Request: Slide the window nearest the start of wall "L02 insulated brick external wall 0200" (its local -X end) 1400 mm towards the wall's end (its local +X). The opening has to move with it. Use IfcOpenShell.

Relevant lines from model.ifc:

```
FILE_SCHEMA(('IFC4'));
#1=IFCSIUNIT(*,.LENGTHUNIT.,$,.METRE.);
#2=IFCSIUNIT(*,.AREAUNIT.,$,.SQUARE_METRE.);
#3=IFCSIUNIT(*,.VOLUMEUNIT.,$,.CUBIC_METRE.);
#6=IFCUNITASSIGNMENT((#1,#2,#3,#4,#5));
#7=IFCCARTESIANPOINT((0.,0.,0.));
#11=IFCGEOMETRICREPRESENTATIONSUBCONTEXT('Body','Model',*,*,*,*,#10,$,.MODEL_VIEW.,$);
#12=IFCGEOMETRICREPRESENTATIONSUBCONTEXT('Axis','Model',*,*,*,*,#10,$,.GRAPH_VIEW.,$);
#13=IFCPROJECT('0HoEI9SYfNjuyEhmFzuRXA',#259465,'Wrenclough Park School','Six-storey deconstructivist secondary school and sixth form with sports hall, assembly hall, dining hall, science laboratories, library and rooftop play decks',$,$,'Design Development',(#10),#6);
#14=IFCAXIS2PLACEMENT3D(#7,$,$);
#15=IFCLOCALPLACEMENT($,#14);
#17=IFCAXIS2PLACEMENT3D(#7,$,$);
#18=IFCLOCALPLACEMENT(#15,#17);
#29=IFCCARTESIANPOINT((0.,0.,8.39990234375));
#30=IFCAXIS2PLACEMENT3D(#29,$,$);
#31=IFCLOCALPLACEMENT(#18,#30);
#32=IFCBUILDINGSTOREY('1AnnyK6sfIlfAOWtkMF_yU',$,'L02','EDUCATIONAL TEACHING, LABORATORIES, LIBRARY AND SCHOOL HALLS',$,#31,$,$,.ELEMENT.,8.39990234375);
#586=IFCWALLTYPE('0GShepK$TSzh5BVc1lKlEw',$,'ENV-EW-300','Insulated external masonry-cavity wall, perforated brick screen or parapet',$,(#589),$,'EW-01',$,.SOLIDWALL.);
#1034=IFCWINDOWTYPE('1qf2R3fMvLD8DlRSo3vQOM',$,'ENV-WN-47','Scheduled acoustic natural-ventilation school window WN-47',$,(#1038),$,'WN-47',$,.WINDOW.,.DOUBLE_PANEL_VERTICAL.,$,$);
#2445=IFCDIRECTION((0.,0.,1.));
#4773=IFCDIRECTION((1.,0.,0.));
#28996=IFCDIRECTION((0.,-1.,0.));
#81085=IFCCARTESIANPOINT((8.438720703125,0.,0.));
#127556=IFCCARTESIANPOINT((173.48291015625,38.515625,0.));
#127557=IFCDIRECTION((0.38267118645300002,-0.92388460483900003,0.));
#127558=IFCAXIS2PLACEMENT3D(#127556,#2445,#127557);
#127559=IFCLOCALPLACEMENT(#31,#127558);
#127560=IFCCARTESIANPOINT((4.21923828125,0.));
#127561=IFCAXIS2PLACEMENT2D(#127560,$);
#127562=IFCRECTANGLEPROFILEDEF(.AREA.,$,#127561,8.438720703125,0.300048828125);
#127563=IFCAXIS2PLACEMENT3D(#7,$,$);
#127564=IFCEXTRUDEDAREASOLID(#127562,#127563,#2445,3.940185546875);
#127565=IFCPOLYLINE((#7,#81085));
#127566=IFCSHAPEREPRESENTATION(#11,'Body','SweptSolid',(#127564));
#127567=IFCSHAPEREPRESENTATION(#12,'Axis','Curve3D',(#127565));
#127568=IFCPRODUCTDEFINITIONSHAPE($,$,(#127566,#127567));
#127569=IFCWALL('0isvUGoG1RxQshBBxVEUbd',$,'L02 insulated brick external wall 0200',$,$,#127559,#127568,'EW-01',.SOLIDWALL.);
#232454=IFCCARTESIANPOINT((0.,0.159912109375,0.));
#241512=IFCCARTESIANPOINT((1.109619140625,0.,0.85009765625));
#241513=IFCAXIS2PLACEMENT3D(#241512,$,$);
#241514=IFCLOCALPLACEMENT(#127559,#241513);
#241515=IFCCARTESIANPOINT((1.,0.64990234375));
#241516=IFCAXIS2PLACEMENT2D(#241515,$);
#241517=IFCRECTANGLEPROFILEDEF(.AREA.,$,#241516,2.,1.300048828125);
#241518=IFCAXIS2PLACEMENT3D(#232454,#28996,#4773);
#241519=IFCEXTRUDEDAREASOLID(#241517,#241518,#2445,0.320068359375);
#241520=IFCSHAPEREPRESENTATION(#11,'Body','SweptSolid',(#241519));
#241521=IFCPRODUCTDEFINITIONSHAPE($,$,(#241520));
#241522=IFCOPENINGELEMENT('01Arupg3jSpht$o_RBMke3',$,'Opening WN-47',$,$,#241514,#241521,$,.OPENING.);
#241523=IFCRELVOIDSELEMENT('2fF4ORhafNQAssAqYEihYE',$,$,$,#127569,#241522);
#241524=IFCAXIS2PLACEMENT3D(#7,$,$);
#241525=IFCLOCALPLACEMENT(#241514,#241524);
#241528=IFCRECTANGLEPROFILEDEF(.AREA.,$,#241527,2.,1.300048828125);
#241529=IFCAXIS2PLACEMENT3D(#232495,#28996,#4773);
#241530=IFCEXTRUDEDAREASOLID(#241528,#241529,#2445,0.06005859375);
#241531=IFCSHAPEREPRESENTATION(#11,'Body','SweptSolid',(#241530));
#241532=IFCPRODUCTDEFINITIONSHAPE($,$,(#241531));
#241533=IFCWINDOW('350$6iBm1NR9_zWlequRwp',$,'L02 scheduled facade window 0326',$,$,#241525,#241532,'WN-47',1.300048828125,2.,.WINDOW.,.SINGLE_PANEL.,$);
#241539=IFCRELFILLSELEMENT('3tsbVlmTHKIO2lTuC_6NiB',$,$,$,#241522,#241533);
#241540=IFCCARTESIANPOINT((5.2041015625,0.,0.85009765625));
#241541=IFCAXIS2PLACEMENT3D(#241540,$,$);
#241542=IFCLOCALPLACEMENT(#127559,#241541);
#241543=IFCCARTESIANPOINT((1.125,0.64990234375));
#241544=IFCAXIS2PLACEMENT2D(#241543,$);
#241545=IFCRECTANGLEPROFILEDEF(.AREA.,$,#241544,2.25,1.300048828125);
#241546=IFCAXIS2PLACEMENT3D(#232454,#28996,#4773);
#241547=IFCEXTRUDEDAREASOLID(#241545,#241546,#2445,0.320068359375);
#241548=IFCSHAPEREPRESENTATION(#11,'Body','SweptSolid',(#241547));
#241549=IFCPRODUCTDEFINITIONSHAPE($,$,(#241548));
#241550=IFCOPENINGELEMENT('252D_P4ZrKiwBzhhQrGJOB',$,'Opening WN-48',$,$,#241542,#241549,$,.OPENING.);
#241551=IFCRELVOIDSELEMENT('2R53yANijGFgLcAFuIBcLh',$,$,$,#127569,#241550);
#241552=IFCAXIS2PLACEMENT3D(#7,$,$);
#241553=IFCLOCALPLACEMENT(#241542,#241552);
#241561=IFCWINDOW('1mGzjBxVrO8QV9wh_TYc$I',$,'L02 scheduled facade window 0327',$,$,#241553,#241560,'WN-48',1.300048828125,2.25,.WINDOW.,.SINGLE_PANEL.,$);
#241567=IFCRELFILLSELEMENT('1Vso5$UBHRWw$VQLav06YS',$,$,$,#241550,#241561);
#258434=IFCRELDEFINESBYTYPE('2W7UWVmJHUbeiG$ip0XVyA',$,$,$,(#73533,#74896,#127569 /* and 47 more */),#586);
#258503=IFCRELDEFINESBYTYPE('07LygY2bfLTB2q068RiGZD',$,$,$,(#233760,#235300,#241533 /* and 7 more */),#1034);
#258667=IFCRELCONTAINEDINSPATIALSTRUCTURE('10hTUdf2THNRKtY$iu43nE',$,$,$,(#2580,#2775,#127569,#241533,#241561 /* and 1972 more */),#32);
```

```python
import ifcopenshell
import ifcopenshell.api.geometry
import ifcopenshell.util.placement

model = ifcopenshell.open("model.ifc")

window = model.by_guid("350$6iBm1NR9_zWlequRwp")
opening = window.FillsVoids[0].RelatingOpeningElement
wall = opening.VoidsElements[0].RelatingBuildingElement

wall_matrix = ifcopenshell.util.placement.get_local_placement(wall.ObjectPlacement)
shift = wall_matrix[:3, 0] * 1.4
before = ifcopenshell.util.placement.get_local_placement(window.ObjectPlacement)[:3, 3].copy()

# The window is placed relative to its opening, so it follows when the opening moves.
matrix = ifcopenshell.util.placement.get_local_placement(opening.ObjectPlacement)
matrix[:3, 3] += shift
ifcopenshell.api.geometry.edit_object_placement(
    model, product=opening, matrix=matrix, is_si=False, should_transform_children=True
)

after = ifcopenshell.util.placement.get_local_placement(window.ObjectPlacement)[:3, 3]
print("window moved by", (after - before).round(3) + 0.0)

model.write("model_updated.ifc")
```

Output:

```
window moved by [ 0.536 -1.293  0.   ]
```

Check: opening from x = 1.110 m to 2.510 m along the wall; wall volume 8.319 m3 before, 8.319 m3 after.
